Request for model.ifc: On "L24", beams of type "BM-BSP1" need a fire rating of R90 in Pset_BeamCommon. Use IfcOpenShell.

First a look at what the model holds.

```python
import ifcopenshell
import ifcopenshell.util.element

model = ifcopenshell.open("model.ifc")
print(model.schema)
storey = next(s for s in model.by_type("IfcBuildingStorey") if s.Name == "L24")
beams = [e for e in ifcopenshell.util.element.get_decomposition(storey) if e.is_a("IfcBeam")]
seen = {}
for e in beams:
    element_type = ifcopenshell.util.element.get_type(e)
    key = (element_type.Name if element_type != e and element_type else None, ifcopenshell.util.element.get_pset(e, "Pset_BeamCommon", "FireRating"))
    seen[key] = seen.get(key, 0) + 1
for (name, value), count in sorted(seen.items(), key=str):
    print(count, "x", name, "|", value)
```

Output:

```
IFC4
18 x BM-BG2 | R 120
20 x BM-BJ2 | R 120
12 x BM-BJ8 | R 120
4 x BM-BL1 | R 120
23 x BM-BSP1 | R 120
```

```python
import ifcopenshell
import ifcopenshell.api.pset
import ifcopenshell.util.element

model = ifcopenshell.open("model.ifc")

storey = next(s for s in model.by_type("IfcBuildingStorey") if s.Name == "L24")
beams = [e for e in ifcopenshell.util.element.get_decomposition(storey) if e.is_a("IfcBeam")]

count = 0
for e in beams:
    element_type = ifcopenshell.util.element.get_type(e)
    if element_type in (None, e) or element_type.Name != "BM-BSP1":
        continue
    found = ifcopenshell.util.element.get_pset(e, "Pset_BeamCommon", should_inherit=False)
    if found:
        pset = model.by_id(found["id"])
        if len(ifcopenshell.util.element.get_elements_by_pset(pset)) > 1:
            pset = ifcopenshell.api.pset.unshare_pset(model, products=[e], pset=pset)[0]
    else:
        pset = ifcopenshell.api.pset.add_pset(model, product=e, name="Pset_BeamCommon")
    ifcopenshell.api.pset.edit_pset(model, pset=pset, properties={"FireRating": "R90"})
    count += 1

print(count, "beams updated")

model.write("model_v2.ifc")
```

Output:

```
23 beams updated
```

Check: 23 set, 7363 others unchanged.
